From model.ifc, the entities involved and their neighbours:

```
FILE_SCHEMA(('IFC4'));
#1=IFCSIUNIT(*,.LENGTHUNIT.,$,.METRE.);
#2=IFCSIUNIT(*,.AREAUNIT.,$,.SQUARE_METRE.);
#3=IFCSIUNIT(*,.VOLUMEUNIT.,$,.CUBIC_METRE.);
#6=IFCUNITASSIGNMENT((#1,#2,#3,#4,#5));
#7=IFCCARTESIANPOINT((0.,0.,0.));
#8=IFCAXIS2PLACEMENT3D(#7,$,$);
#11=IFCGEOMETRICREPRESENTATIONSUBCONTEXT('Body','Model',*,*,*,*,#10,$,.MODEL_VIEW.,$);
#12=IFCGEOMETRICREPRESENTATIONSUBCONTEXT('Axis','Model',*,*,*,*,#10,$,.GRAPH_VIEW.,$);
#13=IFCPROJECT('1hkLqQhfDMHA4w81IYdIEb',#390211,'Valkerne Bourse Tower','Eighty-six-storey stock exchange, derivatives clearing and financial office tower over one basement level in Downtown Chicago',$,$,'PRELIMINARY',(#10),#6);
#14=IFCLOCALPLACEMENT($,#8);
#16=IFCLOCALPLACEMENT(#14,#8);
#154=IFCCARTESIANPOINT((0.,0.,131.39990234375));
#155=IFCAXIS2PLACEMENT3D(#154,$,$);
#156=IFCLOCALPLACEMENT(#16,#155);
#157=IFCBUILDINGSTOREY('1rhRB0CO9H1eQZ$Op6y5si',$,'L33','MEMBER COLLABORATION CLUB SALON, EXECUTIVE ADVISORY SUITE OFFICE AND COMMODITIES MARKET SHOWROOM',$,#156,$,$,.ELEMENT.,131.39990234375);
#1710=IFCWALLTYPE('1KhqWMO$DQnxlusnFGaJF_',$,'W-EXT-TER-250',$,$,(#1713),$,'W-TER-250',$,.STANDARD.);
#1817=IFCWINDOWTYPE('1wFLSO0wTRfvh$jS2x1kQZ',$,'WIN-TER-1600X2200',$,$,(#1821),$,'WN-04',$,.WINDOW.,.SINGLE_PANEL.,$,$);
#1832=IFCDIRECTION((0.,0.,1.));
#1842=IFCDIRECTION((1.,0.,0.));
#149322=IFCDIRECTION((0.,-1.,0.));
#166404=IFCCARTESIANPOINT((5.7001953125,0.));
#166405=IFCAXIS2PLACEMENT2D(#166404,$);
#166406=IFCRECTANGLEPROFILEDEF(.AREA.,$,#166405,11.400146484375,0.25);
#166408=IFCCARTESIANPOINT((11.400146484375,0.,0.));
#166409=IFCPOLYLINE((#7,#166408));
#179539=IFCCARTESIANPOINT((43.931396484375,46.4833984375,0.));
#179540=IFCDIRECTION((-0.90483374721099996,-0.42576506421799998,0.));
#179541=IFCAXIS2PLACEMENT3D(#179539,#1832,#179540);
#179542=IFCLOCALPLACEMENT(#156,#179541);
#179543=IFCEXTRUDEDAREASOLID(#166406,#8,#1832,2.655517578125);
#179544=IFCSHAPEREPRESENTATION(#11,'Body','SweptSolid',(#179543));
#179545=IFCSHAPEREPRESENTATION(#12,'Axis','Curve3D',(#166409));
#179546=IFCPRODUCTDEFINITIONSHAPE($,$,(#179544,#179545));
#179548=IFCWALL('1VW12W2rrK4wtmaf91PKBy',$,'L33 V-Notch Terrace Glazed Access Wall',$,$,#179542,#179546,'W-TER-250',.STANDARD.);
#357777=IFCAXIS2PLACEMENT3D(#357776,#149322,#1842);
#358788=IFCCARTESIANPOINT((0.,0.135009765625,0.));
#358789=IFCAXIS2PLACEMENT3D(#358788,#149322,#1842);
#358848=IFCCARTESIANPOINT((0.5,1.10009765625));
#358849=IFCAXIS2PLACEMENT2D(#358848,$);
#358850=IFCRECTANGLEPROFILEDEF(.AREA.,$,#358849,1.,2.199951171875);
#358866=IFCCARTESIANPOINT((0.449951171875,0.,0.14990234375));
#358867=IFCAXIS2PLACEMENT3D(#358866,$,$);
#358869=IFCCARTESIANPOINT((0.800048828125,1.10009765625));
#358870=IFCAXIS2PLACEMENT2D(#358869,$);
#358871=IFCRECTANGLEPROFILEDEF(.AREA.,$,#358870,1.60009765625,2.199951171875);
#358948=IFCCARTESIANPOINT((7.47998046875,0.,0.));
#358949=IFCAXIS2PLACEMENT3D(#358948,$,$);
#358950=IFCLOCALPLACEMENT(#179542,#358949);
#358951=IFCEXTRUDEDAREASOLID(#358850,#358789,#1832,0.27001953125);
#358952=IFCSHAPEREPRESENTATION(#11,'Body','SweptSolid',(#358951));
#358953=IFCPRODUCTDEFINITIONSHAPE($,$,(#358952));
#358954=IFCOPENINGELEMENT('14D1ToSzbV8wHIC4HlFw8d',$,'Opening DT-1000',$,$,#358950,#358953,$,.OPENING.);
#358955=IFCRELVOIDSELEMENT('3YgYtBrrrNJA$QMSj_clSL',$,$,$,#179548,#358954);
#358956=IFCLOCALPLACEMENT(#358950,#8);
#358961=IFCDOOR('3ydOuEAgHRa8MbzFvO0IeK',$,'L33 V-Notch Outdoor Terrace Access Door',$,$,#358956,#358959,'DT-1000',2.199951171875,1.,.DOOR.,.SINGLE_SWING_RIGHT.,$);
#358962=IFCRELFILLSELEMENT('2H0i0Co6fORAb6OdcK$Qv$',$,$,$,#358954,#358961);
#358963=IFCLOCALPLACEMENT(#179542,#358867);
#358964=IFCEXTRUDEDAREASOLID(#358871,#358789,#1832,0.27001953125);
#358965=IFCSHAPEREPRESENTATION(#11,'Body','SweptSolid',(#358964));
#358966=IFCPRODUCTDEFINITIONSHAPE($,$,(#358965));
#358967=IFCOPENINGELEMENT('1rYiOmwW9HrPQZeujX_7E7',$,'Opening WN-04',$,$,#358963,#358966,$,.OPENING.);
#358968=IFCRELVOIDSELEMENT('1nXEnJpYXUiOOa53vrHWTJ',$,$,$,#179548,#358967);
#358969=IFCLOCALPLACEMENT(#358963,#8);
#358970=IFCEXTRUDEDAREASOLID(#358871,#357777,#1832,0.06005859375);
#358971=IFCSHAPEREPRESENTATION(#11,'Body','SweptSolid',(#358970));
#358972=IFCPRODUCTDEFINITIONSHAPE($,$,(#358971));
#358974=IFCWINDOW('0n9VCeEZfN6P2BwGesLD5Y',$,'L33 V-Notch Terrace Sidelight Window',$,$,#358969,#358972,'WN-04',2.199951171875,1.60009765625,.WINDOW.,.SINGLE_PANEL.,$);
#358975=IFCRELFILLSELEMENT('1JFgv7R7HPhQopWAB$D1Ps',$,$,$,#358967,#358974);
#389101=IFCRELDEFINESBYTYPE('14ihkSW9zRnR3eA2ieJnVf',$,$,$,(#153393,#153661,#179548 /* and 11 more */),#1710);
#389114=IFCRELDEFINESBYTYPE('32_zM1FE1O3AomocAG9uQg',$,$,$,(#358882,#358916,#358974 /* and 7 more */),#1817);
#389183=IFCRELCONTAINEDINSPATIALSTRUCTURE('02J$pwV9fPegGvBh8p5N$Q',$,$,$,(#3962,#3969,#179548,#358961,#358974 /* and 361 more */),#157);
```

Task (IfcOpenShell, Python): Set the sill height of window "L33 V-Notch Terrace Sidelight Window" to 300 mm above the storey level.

```python
import numpy as np
import ifcopenshell
import ifcopenshell.api.geometry
import ifcopenshell.geom
import ifcopenshell.util.element
import ifcopenshell.util.placement
import ifcopenshell.util.shape
import ifcopenshell.util.unit

model = ifcopenshell.open("model.ifc")
unit_scale = ifcopenshell.util.unit.calculate_unit_scale(model)

window = model.by_guid("0n9VCeEZfN6P2BwGesLD5Y")
opening = window.FillsVoids[0].RelatingOpeningElement
storey = ifcopenshell.util.element.get_container(window, ifc_class="IfcBuildingStorey")
level = ifcopenshell.util.placement.get_local_placement(storey.ObjectPlacement)[2, 3]

# The opening's origin need not be at the sill, so measure its lowest point.
shape = ifcopenshell.geom.create_shape(ifcopenshell.geom.settings(), opening)
bottom = ifcopenshell.util.shape.get_shape_bottom_elevation(shape, shape.geometry) / unit_scale
dz = level + 0.3 - bottom

shift = np.array([0.0, 0.0, dz])
# The window is placed relative to its opening, so it follows when the opening moves.
matrix = ifcopenshell.util.placement.get_local_placement(opening.ObjectPlacement)
matrix[:3, 3] += shift
ifcopenshell.api.geometry.edit_object_placement(
    model, product=opening, matrix=matrix, is_si=False, should_transform_children=True
)

print(f"moved by {dz * unit_scale:+.3f} m")

model.write("model-out.ifc")
```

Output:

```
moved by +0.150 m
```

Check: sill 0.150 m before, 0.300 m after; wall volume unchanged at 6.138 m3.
